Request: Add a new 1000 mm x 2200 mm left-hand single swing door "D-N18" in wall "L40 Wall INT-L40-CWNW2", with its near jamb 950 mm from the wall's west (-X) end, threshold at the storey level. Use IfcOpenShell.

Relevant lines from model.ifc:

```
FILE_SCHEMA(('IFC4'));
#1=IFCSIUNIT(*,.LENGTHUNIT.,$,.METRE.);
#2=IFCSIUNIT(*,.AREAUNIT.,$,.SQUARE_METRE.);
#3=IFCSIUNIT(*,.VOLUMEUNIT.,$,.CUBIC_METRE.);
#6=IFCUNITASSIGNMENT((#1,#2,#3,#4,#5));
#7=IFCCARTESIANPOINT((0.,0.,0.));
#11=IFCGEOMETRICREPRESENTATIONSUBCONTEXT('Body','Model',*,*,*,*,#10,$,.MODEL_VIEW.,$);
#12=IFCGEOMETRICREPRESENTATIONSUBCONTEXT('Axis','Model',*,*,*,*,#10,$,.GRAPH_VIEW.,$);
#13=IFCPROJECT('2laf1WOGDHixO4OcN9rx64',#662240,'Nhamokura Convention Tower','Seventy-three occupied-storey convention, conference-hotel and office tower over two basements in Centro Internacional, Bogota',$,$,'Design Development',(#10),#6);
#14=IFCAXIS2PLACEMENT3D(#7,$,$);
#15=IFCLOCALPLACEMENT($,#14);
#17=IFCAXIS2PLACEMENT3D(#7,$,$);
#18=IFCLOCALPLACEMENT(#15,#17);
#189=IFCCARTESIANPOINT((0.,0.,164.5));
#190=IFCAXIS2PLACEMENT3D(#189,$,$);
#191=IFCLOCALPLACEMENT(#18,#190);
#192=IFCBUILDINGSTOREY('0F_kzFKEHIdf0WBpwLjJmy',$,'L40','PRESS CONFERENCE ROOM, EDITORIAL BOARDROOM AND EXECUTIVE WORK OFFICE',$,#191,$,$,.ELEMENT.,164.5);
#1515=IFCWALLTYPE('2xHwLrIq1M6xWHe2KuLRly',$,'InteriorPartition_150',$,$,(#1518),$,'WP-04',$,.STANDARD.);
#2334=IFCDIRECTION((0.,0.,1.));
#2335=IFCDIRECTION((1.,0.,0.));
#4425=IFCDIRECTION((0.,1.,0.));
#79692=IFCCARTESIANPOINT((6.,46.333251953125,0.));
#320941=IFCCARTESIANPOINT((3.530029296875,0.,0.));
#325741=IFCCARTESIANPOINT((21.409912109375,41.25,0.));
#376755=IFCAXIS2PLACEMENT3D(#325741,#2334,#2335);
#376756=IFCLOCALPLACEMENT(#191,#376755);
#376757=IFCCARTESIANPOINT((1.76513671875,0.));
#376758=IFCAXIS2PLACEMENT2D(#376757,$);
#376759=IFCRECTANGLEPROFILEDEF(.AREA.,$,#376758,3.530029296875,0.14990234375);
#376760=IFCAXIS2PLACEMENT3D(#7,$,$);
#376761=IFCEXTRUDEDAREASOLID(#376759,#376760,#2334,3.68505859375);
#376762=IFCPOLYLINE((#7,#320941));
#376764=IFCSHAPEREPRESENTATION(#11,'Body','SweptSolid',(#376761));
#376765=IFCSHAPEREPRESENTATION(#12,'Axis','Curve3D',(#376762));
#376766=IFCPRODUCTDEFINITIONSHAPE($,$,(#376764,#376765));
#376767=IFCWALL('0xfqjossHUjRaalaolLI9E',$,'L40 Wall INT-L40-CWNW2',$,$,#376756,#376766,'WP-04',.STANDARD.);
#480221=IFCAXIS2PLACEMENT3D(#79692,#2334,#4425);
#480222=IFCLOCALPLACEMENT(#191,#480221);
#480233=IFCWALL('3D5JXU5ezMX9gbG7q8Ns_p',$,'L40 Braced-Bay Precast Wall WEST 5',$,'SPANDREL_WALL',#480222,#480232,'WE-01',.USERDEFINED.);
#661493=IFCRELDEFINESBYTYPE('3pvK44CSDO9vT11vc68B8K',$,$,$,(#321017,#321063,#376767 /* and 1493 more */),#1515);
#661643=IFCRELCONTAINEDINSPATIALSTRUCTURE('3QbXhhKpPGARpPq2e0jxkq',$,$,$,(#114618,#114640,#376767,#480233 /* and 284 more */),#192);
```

```python
import numpy as np
import ifcopenshell
import ifcopenshell.api.feature
import ifcopenshell.api.geometry
import ifcopenshell.api.root
import ifcopenshell.api.spatial
import ifcopenshell.geom
import ifcopenshell.util.element
import ifcopenshell.util.placement
import ifcopenshell.util.representation
import ifcopenshell.util.shape
import ifcopenshell.util.unit

model = ifcopenshell.open("model.ifc")
unit_scale = ifcopenshell.util.unit.calculate_unit_scale(model)
settings = ifcopenshell.geom.settings()


def volume(element):
    """Net volume in cubic metres, openings subtracted."""
    shape = ifcopenshell.geom.create_shape(settings, element)
    return ifcopenshell.util.shape.get_volume(shape.geometry)


wall = model.by_id(376767)
storey = ifcopenshell.util.element.get_container(wall, ifc_class="IfcBuildingStorey")
context = ifcopenshell.util.representation.get_context(model, "Model", "Body", "MODEL_VIEW")
before = volume(wall)

width, height, from_end, sill = 1, 2.2, 0.95, 0.0  # metres

# The wall runs along its own X axis, and the end named is its -X end.
wall_shape = ifcopenshell.geom.create_shape(settings, wall)
x, y, z = ifcopenshell.util.shape.get_vertices(wall_shape.geometry).T
start = x.min() + from_end
face, thickness = float(y.min()), float(y.max() - y.min())
wall_matrix = ifcopenshell.util.placement.get_local_placement(wall.ObjectPlacement)
level = ifcopenshell.util.placement.get_local_placement(storey.ObjectPlacement)[2, 3]


def in_wall(x, y):
    """Placement at x, y metres in the wall's axes, at sill height."""
    matrix = wall_matrix.copy()
    matrix[:, 3] = wall_matrix @ np.array([x / unit_scale, y / unit_scale, 0.0, 1.0])
    matrix[2, 3] = level + sill / unit_scale
    return matrix


# Opening: a box that overshoots both wall faces by 50 mm.
opening = ifcopenshell.api.root.create_entity(model, ifc_class="IfcOpeningElement", predefined_type="OPENING")
box = ifcopenshell.api.geometry.add_wall_representation(
    model, context=context, length=width, height=height, thickness=thickness + 0.1
)
ifcopenshell.api.geometry.assign_representation(model, product=opening, representation=box)
ifcopenshell.api.geometry.edit_object_placement(model, product=opening, matrix=in_wall(start, face - 0.05), is_si=False)
ifcopenshell.api.feature.add_feature(model, feature=opening, element=wall)

door = ifcopenshell.api.root.create_entity(model, ifc_class="IfcDoor", name="D-N18", predefined_type="DOOR")
door.OverallWidth, door.OverallHeight = width / unit_scale, height / unit_scale
door.OperationType = "SINGLE_SWING_LEFT"
body = ifcopenshell.api.geometry.add_door_representation(
    model,
    context=context,
    overall_width=door.OverallWidth,
    overall_height=door.OverallHeight,
    operation_type="SINGLE_SWING_LEFT",
    lining_properties={"LiningDepth": thickness / unit_scale, "ThresholdDepth": thickness / unit_scale},
)
ifcopenshell.api.geometry.assign_representation(model, product=door, representation=body)
ifcopenshell.api.spatial.assign_container(model, products=[door], relating_structure=storey)
ifcopenshell.api.feature.add_filling(model, opening=opening, element=door)

# The lining spans the wall, so the door starts at the wall face.
ifcopenshell.api.geometry.edit_object_placement(model, product=door, matrix=in_wall(start, face), is_si=False)

after = volume(wall)

print(f"wall volume {before:.3f} -> {after:.3f} m3")

model.write("model_rev.ifc")
```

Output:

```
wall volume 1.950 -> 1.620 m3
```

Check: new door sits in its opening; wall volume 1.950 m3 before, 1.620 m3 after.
